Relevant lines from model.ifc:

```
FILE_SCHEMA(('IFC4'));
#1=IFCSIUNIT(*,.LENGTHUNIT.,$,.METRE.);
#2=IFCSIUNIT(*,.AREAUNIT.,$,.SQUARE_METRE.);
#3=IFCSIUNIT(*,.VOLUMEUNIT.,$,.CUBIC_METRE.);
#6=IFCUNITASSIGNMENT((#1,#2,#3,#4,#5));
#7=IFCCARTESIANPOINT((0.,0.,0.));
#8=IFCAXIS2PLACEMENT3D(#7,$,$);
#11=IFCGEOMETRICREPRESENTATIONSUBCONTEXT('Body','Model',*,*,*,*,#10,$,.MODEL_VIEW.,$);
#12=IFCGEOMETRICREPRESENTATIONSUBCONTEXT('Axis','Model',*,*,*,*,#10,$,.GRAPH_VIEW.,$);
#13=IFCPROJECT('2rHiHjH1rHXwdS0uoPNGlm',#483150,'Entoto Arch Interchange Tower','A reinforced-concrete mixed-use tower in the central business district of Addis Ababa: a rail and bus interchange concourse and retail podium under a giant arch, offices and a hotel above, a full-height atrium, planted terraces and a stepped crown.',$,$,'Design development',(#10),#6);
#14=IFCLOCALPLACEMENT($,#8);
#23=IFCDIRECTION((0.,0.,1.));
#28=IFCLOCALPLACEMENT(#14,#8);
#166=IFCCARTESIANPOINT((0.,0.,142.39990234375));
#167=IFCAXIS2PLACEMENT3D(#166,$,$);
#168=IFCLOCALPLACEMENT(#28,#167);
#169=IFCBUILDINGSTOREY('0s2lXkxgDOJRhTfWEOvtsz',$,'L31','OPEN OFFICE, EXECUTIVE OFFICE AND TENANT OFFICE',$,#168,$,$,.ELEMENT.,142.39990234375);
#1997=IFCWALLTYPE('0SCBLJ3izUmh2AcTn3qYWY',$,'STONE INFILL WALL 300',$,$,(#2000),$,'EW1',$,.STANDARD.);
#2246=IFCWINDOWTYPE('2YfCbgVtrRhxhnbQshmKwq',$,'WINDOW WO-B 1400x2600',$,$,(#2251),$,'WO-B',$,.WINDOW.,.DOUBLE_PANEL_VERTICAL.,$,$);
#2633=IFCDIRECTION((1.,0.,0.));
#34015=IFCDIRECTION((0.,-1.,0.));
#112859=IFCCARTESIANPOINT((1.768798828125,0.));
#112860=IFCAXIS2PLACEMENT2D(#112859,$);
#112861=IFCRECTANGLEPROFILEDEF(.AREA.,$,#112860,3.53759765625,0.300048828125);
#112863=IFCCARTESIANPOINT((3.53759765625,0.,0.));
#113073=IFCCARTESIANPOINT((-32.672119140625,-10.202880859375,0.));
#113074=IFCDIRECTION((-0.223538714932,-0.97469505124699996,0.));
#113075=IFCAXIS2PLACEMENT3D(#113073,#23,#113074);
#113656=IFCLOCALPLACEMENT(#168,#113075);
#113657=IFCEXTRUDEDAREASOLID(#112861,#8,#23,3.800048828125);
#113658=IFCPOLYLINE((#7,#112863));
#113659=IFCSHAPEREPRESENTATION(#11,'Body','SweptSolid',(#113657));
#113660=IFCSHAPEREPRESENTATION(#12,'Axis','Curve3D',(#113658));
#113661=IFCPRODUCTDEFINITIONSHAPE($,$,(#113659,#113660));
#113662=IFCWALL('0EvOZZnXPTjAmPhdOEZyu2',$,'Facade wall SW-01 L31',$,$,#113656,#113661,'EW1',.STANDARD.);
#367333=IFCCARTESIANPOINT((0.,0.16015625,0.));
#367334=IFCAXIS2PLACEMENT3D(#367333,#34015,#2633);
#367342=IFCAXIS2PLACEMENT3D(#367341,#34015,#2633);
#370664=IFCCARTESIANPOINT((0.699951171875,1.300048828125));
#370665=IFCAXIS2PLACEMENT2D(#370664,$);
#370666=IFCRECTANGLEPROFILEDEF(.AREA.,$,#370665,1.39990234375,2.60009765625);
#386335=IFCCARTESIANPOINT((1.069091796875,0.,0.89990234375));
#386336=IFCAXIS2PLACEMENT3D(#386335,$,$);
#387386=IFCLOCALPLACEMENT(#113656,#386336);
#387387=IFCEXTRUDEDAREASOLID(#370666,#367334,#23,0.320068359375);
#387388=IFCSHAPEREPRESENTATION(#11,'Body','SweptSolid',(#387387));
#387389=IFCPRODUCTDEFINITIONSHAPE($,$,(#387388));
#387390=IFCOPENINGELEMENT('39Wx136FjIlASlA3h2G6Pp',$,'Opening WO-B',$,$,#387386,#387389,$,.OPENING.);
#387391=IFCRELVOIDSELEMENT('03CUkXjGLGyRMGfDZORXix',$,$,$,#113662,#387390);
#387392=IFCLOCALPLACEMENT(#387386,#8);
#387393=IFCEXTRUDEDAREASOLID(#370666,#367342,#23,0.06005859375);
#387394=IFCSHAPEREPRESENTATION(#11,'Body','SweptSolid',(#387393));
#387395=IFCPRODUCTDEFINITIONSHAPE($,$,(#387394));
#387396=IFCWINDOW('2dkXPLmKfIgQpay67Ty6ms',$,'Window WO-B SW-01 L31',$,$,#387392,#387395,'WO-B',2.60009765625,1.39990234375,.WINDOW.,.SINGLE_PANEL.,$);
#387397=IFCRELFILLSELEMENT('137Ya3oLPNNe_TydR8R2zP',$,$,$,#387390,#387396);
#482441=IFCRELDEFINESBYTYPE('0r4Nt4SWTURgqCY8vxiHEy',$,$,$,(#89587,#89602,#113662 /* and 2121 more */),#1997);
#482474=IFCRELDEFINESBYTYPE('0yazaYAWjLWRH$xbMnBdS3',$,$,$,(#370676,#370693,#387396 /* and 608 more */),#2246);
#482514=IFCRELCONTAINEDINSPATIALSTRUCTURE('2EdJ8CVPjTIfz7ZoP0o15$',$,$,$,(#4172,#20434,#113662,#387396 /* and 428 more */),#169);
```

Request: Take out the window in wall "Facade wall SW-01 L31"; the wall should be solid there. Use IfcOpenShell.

```python
import ifcopenshell
import ifcopenshell.api.feature
import ifcopenshell.api.root
import ifcopenshell.geom
import ifcopenshell.util.shape

model = ifcopenshell.open("model.ifc")
settings = ifcopenshell.geom.settings()


def volume(element):
    """Net volume in cubic metres, openings subtracted."""
    shape = ifcopenshell.geom.create_shape(settings, element)
    return ifcopenshell.util.shape.get_volume(shape.geometry)


window = model.by_id(387396)
opening = window.FillsVoids[0].RelatingOpeningElement
wall = opening.VoidsElements[0].RelatingBuildingElement
before = volume(wall)

ifcopenshell.api.root.remove_product(model, product=window)
ifcopenshell.api.feature.remove_feature(model, feature=opening)

after = volume(wall)

print(f"wall volume {before:.3f} -> {after:.3f} m3")

model.write("model_rev.ifc")
```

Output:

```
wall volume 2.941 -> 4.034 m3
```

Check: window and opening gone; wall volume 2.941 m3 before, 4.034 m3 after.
